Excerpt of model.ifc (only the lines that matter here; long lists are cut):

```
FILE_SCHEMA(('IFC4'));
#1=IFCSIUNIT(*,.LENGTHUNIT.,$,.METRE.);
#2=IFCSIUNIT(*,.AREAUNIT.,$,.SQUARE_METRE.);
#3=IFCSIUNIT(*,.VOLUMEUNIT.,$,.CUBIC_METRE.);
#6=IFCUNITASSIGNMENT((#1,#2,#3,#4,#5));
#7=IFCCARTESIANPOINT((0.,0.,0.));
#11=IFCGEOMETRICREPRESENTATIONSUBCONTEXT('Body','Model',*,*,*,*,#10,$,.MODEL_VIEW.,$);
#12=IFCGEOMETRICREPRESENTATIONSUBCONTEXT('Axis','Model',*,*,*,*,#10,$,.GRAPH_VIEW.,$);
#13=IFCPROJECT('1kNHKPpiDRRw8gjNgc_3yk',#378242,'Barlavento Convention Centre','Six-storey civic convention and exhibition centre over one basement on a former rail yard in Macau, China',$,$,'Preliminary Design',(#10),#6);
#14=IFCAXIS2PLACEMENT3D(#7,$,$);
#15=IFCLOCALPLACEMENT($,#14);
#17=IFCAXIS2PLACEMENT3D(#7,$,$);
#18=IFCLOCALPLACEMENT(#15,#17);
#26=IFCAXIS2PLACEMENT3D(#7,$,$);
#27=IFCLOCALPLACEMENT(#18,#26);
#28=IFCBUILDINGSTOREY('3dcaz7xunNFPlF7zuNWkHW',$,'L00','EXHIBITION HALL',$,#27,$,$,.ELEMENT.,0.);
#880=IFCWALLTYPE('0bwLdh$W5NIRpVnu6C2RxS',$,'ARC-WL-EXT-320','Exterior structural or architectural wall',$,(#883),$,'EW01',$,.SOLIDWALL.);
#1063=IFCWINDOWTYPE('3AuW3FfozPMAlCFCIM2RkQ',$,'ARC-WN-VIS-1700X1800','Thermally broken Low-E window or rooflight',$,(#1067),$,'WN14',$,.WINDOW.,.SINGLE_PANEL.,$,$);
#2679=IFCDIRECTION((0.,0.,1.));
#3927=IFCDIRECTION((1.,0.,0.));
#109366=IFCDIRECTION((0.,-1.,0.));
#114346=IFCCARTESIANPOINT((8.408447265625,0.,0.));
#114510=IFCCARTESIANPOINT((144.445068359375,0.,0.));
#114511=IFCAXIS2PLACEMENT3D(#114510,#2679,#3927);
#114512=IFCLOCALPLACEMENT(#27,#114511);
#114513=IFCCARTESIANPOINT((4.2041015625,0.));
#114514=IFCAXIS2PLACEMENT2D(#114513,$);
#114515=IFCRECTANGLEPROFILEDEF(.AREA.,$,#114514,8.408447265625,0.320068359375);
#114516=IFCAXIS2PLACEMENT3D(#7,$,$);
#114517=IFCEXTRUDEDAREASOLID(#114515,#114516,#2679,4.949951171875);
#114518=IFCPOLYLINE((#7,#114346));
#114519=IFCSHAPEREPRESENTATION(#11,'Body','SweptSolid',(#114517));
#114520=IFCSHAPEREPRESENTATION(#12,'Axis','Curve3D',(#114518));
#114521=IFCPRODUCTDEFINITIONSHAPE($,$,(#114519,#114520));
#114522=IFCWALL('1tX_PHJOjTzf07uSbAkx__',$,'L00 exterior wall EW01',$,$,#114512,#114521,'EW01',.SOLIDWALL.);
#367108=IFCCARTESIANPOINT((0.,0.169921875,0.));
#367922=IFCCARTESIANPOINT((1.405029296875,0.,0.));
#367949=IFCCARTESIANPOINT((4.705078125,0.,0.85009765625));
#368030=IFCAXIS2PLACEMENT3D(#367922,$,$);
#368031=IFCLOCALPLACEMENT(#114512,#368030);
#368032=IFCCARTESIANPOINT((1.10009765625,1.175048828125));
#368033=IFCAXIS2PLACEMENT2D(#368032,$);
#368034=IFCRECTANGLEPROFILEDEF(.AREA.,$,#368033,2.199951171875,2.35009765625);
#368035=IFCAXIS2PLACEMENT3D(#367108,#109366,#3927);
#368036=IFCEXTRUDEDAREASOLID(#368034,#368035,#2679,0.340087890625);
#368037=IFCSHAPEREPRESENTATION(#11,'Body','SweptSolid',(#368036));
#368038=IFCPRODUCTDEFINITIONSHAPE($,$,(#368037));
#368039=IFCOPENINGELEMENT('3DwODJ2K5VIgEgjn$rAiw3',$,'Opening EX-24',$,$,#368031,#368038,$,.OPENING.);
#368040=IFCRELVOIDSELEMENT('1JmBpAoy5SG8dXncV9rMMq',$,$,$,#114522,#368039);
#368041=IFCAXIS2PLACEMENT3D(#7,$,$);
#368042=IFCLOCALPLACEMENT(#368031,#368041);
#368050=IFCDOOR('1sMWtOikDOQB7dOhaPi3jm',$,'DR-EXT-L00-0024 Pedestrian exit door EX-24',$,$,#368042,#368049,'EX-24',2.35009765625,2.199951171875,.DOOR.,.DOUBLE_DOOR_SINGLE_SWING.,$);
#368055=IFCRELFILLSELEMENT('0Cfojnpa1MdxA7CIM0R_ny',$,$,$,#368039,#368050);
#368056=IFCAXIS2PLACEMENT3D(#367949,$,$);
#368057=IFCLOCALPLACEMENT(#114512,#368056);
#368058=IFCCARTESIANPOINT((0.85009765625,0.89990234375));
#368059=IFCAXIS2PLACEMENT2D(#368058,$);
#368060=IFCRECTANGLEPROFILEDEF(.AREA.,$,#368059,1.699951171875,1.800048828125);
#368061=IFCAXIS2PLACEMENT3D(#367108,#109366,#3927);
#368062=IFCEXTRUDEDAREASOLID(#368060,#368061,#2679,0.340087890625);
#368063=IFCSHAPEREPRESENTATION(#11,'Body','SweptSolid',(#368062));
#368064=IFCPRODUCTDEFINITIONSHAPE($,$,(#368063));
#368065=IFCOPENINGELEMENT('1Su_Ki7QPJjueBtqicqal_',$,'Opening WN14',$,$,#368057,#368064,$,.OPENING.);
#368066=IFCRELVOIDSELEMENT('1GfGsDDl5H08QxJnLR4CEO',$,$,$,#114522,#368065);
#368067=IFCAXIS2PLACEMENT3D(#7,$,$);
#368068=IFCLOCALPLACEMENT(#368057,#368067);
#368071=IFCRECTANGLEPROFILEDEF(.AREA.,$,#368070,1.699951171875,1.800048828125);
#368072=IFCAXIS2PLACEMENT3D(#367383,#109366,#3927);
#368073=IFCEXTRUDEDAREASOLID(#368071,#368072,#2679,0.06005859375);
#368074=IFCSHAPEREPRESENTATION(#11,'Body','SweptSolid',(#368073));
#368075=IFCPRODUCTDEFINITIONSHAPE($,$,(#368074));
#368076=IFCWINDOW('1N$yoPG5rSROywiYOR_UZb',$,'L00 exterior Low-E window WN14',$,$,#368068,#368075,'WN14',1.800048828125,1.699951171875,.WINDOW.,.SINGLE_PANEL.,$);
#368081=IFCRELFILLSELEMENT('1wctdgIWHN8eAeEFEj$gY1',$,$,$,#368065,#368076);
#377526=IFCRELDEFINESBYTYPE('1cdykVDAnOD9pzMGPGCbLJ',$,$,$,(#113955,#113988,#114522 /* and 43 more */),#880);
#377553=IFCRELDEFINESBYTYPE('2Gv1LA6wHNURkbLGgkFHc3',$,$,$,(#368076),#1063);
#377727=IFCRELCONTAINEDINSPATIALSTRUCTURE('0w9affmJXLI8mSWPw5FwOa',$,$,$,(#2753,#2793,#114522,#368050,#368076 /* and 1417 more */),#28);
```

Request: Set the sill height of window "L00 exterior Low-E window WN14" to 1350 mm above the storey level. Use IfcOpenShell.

```python
import numpy as np
import ifcopenshell
import ifcopenshell.api.geometry
import ifcopenshell.geom
import ifcopenshell.util.element
import ifcopenshell.util.placement
import ifcopenshell.util.shape
import ifcopenshell.util.unit

model = ifcopenshell.open("model.ifc")
unit_scale = ifcopenshell.util.unit.calculate_unit_scale(model)

window = model.by_guid("1N$yoPG5rSROywiYOR_UZb")
opening = window.FillsVoids[0].RelatingOpeningElement
storey = ifcopenshell.util.element.get_container(window, ifc_class="IfcBuildingStorey")
level = ifcopenshell.util.placement.get_local_placement(storey.ObjectPlacement)[2, 3]

# The opening's origin need not be at the sill, so measure its lowest point.
shape = ifcopenshell.geom.create_shape(ifcopenshell.geom.settings(), opening)
bottom = ifcopenshell.util.shape.get_shape_bottom_elevation(shape, shape.geometry) / unit_scale
dz = level + 1.35 / unit_scale - bottom

shift = np.array([0.0, 0.0, dz])
# The window is placed relative to its opening, so it follows when the opening moves.
matrix = ifcopenshell.util.placement.get_local_placement(opening.ObjectPlacement)
matrix[:3, 3] += shift
ifcopenshell.api.geometry.edit_object_placement(
    model, product=opening, matrix=matrix, is_si=False, should_transform_children=True
)

print(f"moved by {dz * unit_scale:+.3f} m")

model.write("model_edited.ifc")
```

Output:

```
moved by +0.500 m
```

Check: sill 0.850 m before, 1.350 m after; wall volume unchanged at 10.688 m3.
